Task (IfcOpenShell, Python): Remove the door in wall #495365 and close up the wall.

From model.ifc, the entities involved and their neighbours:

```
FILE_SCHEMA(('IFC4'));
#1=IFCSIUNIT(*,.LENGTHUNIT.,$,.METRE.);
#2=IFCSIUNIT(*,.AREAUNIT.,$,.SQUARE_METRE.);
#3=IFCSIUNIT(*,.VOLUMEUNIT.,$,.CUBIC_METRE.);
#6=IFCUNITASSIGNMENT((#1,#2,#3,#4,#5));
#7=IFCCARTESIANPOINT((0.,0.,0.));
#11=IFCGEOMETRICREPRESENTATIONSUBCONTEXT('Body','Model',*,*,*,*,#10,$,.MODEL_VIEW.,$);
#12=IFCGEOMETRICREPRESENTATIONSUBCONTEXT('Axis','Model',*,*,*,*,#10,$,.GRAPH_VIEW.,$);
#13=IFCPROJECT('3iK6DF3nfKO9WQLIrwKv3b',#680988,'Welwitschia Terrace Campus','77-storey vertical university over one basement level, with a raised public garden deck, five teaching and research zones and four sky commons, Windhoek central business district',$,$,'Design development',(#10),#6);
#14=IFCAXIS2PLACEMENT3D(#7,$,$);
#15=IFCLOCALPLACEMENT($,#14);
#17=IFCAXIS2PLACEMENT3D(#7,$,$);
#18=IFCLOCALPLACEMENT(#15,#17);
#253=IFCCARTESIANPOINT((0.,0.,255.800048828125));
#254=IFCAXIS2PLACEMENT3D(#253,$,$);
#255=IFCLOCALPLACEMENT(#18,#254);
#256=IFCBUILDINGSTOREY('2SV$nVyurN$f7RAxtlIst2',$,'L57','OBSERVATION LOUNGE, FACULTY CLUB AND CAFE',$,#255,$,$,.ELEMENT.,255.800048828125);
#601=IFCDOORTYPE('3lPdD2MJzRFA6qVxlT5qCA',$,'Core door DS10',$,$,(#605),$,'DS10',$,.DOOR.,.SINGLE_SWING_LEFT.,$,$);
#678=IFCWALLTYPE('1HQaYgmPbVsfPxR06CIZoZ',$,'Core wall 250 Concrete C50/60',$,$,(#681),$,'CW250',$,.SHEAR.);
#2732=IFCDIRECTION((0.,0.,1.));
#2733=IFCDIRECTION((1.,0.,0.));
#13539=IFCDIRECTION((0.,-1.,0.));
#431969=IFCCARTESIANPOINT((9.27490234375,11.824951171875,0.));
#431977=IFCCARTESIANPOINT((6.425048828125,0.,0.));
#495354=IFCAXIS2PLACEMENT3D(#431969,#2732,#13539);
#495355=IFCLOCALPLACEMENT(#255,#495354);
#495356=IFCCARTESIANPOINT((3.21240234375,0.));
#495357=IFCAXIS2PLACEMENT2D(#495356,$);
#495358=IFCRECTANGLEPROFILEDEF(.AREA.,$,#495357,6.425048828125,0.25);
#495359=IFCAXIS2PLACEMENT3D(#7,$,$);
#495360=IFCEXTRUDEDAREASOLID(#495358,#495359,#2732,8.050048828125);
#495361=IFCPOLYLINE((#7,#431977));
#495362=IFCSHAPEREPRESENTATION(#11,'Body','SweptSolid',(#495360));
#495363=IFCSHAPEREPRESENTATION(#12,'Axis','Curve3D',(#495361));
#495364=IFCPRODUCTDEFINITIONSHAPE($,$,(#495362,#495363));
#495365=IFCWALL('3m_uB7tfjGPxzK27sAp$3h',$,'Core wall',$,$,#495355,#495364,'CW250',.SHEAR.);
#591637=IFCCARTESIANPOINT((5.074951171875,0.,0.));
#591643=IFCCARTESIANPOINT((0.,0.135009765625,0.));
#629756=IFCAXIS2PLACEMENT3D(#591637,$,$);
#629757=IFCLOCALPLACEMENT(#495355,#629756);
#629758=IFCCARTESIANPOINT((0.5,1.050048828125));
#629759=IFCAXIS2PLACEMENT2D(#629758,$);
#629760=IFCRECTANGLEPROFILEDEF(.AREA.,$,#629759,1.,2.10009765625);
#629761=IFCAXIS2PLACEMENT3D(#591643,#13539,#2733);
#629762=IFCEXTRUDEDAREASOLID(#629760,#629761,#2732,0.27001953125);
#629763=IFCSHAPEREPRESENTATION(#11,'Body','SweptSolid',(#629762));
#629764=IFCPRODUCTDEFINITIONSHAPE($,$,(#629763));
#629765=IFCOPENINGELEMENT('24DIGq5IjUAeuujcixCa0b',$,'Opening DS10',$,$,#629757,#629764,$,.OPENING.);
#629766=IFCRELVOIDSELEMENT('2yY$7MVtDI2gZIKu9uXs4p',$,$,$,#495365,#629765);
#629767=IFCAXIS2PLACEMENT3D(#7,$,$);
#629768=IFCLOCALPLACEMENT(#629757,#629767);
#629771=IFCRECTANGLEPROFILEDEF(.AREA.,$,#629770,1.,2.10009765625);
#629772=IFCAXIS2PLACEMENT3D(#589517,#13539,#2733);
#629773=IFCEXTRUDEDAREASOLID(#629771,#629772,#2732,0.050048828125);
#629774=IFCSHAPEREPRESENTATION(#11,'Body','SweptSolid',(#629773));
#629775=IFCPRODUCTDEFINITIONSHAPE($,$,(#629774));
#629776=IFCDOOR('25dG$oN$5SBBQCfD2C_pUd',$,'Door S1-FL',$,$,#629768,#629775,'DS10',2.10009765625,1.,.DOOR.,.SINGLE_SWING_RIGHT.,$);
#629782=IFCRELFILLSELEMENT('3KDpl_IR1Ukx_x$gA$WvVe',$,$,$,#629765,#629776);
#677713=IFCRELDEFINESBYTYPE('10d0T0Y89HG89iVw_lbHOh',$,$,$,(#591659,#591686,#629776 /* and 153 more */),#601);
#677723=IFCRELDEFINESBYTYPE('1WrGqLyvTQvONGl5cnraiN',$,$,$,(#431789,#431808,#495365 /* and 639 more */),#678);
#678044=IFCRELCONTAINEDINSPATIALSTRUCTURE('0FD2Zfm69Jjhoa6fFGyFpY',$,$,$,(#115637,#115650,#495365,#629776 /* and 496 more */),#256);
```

```python
import ifcopenshell
import ifcopenshell.api.feature
import ifcopenshell.api.root
import ifcopenshell.geom
import ifcopenshell.util.shape

model = ifcopenshell.open("model.ifc")
settings = ifcopenshell.geom.settings()


def volume(element):
    """Net volume in cubic metres, openings subtracted."""
    shape = ifcopenshell.geom.create_shape(settings, element)
    return ifcopenshell.util.shape.get_volume(shape.geometry)


door = model.by_guid("25dG$oN$5SBBQCfD2C_pUd")
opening = door.FillsVoids[0].RelatingOpeningElement
wall = opening.VoidsElements[0].RelatingBuildingElement
before = volume(wall)

ifcopenshell.api.root.remove_product(model, product=door)
ifcopenshell.api.feature.remove_feature(model, feature=opening)

after = volume(wall)

print(f"wall volume {before:.3f} -> {after:.3f} m3")

model.write("model_updated.ifc")
```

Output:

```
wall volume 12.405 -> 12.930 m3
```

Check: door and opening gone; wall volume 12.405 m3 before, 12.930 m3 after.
